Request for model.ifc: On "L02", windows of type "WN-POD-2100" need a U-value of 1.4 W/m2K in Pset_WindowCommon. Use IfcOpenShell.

First a look at what the model holds.

```python
import ifcopenshell
import ifcopenshell.util.element

model = ifcopenshell.open("model.ifc")
print(model.schema)
storey = next(s for s in model.by_type("IfcBuildingStorey") if s.Name == "L02")
windows = [e for e in ifcopenshell.util.element.get_decomposition(storey) if e.is_a("IfcWindow")]
seen = {}
for e in windows:
    element_type = ifcopenshell.util.element.get_type(e)
    key = (element_type.Name if element_type != e and element_type else None, ifcopenshell.util.element.get_pset(e, "Pset_WindowCommon", "ThermalTransmittance"))
    seen[key] = seen.get(key, 0) + 1
for (name, value), count in sorted(seen.items(), key=str):
    print(count, "x", name, "|", value)
```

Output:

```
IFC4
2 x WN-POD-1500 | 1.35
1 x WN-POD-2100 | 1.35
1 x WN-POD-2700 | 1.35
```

```python
import ifcopenshell
import ifcopenshell.api.pset
import ifcopenshell.util.element

model = ifcopenshell.open("model.ifc")

storey = next(s for s in model.by_type("IfcBuildingStorey") if s.Name == "L02")
windows = [e for e in ifcopenshell.util.element.get_decomposition(storey) if e.is_a("IfcWindow")]

count = 0
for e in windows:
    element_type = ifcopenshell.util.element.get_type(e)
    if element_type in (None, e) or element_type.Name != "WN-POD-2100":
        continue
    # add_pset returns the element's existing set when there is one.
    pset = ifcopenshell.api.pset.add_pset(model, product=e, name="Pset_WindowCommon")
    ifcopenshell.api.pset.edit_pset(model, pset=pset, properties={"ThermalTransmittance": 1.4})
    count += 1

print(count, "windows updated")

model.write("model_v2.ifc")
```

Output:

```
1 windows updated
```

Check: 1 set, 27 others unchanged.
